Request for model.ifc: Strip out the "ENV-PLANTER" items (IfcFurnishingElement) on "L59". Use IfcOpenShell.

First a look at what the model holds.

```python
import ifcopenshell
import ifcopenshell.util.element

model = ifcopenshell.open("model.ifc")
print(model.schema)
storey = next(s for s in model.by_type("IfcBuildingStorey") if s.Name == "L59")
furniture = [e for e in ifcopenshell.util.element.get_decomposition(storey) if e.is_a("IfcFurnishingElement")]
seen = {}
for e in furniture:
    element_type = ifcopenshell.util.element.get_type(e)
    name = element_type.Name if element_type not in (None, e) else None
    seen[name] = seen.get(name, 0) + 1
for name, count in sorted(seen.items(), key=str):
    print(count, "x", name)
```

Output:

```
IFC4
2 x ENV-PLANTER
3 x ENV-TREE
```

```python
import ifcopenshell
import ifcopenshell.api.root
import ifcopenshell.util.element

model = ifcopenshell.open("model.ifc")

storey = next(s for s in model.by_type("IfcBuildingStorey") if s.Name == "L59")
furniture = [e for e in ifcopenshell.util.element.get_decomposition(storey) if e.is_a("IfcFurnishingElement")]
targets = [e for e in furniture if (t := ifcopenshell.util.element.get_type(e)) not in (None, e) and t.Name == "ENV-PLANTER"]

for e in targets:
    ifcopenshell.api.root.remove_product(model, product=e)
print(len(targets), "removed")

model.write("model-out.ifc")
```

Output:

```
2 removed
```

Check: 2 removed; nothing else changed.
